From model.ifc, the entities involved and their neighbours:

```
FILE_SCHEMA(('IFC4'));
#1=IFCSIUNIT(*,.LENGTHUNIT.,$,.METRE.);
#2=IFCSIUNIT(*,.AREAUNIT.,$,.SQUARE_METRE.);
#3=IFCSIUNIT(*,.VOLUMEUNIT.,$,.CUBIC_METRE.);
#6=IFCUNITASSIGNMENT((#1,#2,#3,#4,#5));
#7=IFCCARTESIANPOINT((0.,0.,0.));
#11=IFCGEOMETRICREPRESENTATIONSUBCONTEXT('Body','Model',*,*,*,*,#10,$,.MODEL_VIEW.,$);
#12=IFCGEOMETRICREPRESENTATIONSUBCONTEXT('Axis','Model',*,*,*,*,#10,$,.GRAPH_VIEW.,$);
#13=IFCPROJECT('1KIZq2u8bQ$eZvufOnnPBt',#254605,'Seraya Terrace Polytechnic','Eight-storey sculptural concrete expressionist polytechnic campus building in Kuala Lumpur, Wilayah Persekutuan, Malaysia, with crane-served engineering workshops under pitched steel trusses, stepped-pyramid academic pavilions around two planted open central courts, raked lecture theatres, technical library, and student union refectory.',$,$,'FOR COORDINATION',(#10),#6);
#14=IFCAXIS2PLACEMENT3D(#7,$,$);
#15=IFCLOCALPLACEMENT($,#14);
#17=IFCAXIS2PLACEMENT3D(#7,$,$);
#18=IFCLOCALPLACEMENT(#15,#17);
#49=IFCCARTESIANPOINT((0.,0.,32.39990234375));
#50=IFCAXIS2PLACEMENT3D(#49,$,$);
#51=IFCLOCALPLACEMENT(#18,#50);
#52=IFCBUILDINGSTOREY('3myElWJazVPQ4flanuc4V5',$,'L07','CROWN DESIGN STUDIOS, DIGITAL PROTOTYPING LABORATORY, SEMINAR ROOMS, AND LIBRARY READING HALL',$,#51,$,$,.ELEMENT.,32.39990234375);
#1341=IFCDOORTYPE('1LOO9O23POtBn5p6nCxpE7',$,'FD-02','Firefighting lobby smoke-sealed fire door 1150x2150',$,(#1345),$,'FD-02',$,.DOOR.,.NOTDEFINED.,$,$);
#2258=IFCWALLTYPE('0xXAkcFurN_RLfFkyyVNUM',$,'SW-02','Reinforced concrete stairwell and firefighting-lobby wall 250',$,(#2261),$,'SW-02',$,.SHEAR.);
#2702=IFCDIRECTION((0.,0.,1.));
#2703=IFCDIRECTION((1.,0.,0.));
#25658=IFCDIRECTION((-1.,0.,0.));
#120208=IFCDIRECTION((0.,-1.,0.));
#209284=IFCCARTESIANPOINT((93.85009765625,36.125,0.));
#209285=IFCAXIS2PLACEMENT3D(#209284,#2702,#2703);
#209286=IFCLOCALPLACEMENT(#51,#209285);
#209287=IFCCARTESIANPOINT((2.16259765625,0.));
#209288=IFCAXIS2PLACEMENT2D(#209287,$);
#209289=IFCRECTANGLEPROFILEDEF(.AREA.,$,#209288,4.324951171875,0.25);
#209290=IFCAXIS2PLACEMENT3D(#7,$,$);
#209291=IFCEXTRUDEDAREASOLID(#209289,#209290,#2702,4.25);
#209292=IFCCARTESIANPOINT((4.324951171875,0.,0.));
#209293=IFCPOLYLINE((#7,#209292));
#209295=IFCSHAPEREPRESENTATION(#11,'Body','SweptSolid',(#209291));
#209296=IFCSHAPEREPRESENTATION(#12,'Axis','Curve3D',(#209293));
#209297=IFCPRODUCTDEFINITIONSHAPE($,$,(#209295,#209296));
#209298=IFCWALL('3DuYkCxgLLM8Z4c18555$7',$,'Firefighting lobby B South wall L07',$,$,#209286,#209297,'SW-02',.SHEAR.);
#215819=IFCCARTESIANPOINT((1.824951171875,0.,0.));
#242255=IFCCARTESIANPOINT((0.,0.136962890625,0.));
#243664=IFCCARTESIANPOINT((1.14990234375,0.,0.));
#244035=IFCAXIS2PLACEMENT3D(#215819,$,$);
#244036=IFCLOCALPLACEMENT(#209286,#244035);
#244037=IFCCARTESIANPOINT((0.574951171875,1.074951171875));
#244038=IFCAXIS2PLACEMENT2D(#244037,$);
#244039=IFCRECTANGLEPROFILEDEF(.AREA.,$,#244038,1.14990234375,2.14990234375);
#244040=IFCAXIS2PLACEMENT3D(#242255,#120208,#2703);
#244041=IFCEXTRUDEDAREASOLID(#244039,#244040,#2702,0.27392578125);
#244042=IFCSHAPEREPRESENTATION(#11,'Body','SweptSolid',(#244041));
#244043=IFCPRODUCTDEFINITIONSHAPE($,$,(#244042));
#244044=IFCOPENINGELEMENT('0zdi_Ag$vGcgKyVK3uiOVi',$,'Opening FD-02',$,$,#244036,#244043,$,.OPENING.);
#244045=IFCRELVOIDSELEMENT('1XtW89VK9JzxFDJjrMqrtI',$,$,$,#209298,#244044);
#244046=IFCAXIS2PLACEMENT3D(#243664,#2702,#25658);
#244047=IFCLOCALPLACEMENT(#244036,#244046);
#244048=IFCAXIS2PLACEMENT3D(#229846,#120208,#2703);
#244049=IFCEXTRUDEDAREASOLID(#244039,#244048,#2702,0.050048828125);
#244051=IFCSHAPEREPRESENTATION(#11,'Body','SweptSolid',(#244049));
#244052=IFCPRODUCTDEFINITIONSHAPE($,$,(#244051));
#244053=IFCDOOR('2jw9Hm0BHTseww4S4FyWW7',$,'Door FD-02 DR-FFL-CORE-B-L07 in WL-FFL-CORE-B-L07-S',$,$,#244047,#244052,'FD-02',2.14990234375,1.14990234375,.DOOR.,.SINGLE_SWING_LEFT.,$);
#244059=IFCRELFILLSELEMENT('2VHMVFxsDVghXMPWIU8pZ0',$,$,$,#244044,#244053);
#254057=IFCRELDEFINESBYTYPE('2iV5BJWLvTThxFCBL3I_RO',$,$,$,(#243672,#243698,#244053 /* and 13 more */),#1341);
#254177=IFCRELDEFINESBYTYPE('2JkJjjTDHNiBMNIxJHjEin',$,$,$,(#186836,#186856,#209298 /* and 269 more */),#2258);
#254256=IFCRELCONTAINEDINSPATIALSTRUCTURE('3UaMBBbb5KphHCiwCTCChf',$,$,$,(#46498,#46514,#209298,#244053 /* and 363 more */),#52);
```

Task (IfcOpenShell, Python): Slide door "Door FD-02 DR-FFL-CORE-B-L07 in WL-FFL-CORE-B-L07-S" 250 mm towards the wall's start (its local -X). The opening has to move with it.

```python
import ifcopenshell
import ifcopenshell.api.geometry
import ifcopenshell.util.placement

model = ifcopenshell.open("model.ifc")

door = model.by_guid("2jw9Hm0BHTseww4S4FyWW7")
opening = door.FillsVoids[0].RelatingOpeningElement
wall = opening.VoidsElements[0].RelatingBuildingElement

wall_matrix = ifcopenshell.util.placement.get_local_placement(wall.ObjectPlacement)
shift = wall_matrix[:3, 0] * -0.25
before = ifcopenshell.util.placement.get_local_placement(door.ObjectPlacement)[:3, 3].copy()

# The door is placed relative to its opening, so it follows when the opening moves.
matrix = ifcopenshell.util.placement.get_local_placement(opening.ObjectPlacement)
matrix[:3, 3] += shift
ifcopenshell.api.geometry.edit_object_placement(
    model, product=opening, matrix=matrix, is_si=False, should_transform_children=True
)

after = ifcopenshell.util.placement.get_local_placement(door.ObjectPlacement)[:3, 3]
print("door moved by", (after - before).round(3) + 0.0)

model.write("model-out.ifc")
```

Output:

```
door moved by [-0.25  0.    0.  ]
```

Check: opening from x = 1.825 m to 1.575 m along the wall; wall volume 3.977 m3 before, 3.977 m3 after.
